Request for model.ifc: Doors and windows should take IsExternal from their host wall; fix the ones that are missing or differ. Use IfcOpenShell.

First a look at what the model holds.

```python
import ifcopenshell
import ifcopenshell.util.element

model = ifcopenshell.open("model.ifc")
print(model.schema)
seen = {}
for e in model.by_type("IfcDoor") + model.by_type("IfcWindow"):
    if not e.FillsVoids:
        continue
    host = e.FillsVoids[0].RelatingOpeningElement.VoidsElements[0].RelatingBuildingElement
    own = ifcopenshell.util.element.get_pset(e, f"Pset_{e.is_a()[3:].removesuffix('StandardCase')}Common", "IsExternal")
    wall = ifcopenshell.util.element.get_pset(host, "Pset_WallCommon", "IsExternal")
    seen[e.is_a(), own, wall] = seen.get((e.is_a(), own, wall), 0) + 1
for (cls, own, wall), count in sorted(seen.items(), key=str):
    print(count, cls, "IsExternal:", own, "| host wall:", wall)
```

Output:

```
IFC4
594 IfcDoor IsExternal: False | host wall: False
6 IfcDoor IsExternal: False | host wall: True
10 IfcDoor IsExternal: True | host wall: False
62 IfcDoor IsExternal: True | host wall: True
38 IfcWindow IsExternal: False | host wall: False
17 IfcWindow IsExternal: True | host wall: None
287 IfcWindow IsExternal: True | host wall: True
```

```python
import ifcopenshell
import ifcopenshell.api.pset
import ifcopenshell.util.element

model = ifcopenshell.open("model.ifc")

count = 0
for ifc_class, pset_name in (("IfcDoor", "Pset_DoorCommon"), ("IfcWindow", "Pset_WindowCommon")):
    for e in model.by_type(ifc_class):
        if not e.FillsVoids:
            continue
        host = e.FillsVoids[0].RelatingOpeningElement.VoidsElements[0].RelatingBuildingElement
        external = ifcopenshell.util.element.get_pset(host, "Pset_WallCommon", "IsExternal")
        if external is None or ifcopenshell.util.element.get_pset(e, pset_name, "IsExternal") == external:
            continue
        pset = ifcopenshell.api.pset.add_pset(model, product=e, name=pset_name)
        ifcopenshell.api.pset.edit_pset(model, pset=pset, properties={"IsExternal": external})
        count += 1

print(count, "updated")

model.write("model_v2.ifc")
```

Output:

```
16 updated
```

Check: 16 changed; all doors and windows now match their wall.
